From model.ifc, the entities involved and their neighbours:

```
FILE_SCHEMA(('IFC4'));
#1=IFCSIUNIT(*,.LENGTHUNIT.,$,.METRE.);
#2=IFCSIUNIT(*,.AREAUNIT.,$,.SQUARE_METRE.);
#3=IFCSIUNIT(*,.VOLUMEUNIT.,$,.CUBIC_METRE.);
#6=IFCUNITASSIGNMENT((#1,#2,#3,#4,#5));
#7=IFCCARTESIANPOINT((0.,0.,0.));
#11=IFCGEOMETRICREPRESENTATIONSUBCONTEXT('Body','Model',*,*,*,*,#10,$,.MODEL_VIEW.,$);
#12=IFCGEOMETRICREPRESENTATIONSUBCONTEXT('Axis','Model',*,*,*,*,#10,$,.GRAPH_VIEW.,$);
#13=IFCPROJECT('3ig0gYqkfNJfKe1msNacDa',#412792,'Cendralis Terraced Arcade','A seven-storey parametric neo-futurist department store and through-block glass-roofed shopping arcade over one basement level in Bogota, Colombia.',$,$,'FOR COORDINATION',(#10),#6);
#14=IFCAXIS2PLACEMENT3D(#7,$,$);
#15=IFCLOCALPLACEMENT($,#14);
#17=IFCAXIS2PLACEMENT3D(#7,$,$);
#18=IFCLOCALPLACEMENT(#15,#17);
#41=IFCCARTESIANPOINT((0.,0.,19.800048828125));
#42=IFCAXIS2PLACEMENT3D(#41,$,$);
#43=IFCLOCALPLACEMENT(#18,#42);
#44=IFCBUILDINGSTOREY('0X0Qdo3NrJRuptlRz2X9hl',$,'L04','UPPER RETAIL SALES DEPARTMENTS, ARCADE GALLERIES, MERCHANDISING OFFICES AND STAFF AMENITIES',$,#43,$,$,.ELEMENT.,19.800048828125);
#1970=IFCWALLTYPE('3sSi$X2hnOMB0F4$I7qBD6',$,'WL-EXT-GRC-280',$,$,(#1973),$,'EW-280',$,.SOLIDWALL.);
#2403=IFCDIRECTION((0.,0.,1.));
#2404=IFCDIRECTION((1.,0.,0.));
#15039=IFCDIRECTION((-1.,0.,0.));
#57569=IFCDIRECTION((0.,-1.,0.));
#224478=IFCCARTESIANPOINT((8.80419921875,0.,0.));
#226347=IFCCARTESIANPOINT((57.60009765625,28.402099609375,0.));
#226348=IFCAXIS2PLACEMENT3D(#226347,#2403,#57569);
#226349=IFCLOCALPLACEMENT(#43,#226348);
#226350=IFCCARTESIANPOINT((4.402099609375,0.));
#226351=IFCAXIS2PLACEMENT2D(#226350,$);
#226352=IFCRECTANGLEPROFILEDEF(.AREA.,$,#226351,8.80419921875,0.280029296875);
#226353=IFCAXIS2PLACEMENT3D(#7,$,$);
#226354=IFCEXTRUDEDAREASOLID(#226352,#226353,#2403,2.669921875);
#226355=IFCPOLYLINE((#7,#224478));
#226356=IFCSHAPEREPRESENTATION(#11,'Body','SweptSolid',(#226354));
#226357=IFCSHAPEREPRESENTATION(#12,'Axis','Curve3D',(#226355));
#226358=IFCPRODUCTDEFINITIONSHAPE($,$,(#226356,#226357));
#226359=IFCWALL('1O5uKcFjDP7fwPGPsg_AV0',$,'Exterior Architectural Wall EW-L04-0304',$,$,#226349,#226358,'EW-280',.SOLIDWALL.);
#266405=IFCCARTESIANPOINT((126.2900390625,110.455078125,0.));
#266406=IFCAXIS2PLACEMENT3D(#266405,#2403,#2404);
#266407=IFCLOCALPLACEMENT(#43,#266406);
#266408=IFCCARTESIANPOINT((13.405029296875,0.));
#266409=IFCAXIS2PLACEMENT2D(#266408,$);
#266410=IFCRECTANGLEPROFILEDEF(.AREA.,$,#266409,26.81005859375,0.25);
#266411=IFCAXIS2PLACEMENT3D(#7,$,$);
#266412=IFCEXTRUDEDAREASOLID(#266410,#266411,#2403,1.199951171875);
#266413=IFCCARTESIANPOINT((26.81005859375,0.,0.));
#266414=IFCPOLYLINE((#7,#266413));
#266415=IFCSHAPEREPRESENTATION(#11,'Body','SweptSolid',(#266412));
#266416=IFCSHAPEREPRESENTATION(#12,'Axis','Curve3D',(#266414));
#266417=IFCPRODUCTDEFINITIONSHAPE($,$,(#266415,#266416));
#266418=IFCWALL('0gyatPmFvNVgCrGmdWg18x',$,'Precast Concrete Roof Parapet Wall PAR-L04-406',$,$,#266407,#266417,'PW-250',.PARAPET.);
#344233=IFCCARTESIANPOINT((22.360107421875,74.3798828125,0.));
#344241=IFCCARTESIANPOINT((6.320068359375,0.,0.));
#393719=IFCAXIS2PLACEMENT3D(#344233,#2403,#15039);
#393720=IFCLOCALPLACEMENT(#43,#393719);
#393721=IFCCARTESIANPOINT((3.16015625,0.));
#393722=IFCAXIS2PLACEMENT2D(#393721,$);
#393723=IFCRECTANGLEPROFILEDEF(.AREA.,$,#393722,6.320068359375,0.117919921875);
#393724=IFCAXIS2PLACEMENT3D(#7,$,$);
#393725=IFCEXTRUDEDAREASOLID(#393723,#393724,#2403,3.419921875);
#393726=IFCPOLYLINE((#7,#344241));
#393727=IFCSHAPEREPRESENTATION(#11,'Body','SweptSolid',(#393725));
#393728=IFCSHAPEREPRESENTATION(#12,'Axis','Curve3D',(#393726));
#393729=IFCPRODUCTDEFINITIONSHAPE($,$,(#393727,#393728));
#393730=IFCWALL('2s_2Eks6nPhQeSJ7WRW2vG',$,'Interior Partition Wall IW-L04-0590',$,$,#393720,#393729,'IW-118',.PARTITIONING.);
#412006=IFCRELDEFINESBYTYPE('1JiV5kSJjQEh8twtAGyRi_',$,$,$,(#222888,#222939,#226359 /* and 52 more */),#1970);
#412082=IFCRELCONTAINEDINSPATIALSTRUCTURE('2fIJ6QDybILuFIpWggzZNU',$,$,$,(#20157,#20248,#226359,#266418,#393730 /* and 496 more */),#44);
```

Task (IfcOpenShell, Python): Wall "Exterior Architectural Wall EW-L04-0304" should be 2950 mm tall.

```python
import ifcopenshell
import ifcopenshell.geom
import ifcopenshell.util.representation
import ifcopenshell.util.shape

model = ifcopenshell.open("model.ifc")
settings = ifcopenshell.geom.settings()


def volume(element):
    """Net volume in cubic metres, openings subtracted."""
    shape = ifcopenshell.geom.create_shape(settings, element)
    return ifcopenshell.util.shape.get_volume(shape.geometry)


wall = model.by_guid("1O5uKcFjDP7fwPGPsg_AV0")
before = volume(wall)

body = ifcopenshell.util.representation.get_representation(wall, "Model", "Body")
solid = body.Items[0]
old_height = solid.Depth
solid.Depth = 2.95
after = volume(wall)

print(f"height {old_height:g} -> {solid.Depth:g}, volume {before:.3f} -> {after:.3f} m3")

model.write("model_updated.ifc")
```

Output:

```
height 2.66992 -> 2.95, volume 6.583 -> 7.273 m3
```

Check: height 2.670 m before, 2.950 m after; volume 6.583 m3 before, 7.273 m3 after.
